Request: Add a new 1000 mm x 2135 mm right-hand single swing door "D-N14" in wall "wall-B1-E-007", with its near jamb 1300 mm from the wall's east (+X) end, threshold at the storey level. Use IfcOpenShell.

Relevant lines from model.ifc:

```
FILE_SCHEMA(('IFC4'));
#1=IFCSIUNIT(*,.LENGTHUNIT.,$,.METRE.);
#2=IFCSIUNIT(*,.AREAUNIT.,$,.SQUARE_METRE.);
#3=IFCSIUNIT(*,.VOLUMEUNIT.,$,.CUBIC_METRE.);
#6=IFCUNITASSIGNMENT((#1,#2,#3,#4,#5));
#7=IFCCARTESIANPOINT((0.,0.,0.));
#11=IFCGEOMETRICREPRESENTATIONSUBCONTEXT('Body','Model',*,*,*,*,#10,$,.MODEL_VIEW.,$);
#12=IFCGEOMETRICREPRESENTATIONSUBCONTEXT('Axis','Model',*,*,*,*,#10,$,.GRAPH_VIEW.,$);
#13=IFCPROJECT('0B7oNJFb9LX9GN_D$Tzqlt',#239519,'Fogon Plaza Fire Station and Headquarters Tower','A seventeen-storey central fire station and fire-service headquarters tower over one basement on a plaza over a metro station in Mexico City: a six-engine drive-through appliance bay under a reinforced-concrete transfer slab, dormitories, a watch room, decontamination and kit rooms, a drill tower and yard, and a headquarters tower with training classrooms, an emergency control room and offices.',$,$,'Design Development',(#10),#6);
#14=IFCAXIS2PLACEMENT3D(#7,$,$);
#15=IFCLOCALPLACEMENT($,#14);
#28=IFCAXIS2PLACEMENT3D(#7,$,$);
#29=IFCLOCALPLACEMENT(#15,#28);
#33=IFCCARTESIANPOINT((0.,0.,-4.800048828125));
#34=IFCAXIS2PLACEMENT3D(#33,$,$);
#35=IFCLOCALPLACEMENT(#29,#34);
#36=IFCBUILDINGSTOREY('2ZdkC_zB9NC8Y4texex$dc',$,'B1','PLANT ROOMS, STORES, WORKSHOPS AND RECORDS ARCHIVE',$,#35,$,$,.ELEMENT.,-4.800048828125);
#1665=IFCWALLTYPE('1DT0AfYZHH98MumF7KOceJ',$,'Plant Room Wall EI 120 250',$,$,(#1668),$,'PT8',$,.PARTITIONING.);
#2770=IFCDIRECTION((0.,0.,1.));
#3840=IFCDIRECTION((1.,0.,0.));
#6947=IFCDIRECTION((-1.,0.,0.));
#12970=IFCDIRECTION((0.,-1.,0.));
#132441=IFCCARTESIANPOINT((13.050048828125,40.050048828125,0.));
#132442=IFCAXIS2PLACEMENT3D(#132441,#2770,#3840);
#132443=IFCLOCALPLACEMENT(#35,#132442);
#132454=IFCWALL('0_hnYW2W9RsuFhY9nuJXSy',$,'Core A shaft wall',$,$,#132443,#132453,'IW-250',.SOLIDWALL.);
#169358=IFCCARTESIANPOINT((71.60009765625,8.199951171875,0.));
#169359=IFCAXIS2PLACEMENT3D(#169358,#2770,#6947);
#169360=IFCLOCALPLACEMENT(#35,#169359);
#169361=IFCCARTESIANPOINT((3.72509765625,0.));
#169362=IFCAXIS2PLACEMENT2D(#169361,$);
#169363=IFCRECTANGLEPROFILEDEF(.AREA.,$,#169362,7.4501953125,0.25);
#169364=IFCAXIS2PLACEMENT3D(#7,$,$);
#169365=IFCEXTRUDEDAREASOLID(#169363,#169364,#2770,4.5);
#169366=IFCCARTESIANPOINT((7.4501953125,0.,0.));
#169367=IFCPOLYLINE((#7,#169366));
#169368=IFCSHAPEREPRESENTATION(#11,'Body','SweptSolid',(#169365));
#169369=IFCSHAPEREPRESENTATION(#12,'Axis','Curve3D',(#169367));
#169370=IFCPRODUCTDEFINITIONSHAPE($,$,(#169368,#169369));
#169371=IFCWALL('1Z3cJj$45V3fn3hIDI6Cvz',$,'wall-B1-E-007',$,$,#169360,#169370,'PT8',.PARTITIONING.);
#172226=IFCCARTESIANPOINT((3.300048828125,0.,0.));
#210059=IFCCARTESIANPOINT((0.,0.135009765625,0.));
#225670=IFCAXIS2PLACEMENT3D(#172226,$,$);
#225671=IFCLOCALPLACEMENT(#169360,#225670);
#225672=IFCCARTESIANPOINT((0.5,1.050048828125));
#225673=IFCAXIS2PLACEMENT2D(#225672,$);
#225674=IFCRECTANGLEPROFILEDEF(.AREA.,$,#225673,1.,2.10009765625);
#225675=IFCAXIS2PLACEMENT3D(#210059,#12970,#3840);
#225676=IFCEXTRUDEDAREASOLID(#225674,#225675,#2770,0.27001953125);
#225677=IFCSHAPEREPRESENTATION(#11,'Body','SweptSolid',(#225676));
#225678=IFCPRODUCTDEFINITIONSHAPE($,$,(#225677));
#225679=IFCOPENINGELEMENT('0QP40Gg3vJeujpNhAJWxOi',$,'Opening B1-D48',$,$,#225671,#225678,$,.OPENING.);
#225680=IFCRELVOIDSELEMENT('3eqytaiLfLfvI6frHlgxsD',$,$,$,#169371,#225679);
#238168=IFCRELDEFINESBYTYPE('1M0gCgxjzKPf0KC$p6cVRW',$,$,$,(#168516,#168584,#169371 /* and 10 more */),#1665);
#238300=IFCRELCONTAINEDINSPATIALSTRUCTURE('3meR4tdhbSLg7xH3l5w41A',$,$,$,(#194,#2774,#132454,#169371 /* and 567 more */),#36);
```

```python
import numpy as np
import ifcopenshell
import ifcopenshell.api.feature
import ifcopenshell.api.geometry
import ifcopenshell.api.root
import ifcopenshell.api.spatial
import ifcopenshell.geom
import ifcopenshell.util.element
import ifcopenshell.util.placement
import ifcopenshell.util.representation
import ifcopenshell.util.shape
import ifcopenshell.util.unit

model = ifcopenshell.open("model.ifc")
unit_scale = ifcopenshell.util.unit.calculate_unit_scale(model)
settings = ifcopenshell.geom.settings()


def volume(element):
    """Net volume in cubic metres, openings subtracted."""
    shape = ifcopenshell.geom.create_shape(settings, element)
    return ifcopenshell.util.shape.get_volume(shape.geometry)


wall = model.by_guid("1Z3cJj$45V3fn3hIDI6Cvz")
storey = ifcopenshell.util.element.get_container(wall, ifc_class="IfcBuildingStorey")
context = ifcopenshell.util.representation.get_context(model, "Model", "Body", "MODEL_VIEW")
before = volume(wall)

width, height, from_end, sill = 1, 2.135, 1.3, 0.0  # metres

# The wall runs along its own X axis, and the end named is its -X end.
wall_shape = ifcopenshell.geom.create_shape(settings, wall)
x, y, z = ifcopenshell.util.shape.get_vertices(wall_shape.geometry).T
start = x.min() + from_end
face, thickness = float(y.min()), float(y.max() - y.min())
wall_matrix = ifcopenshell.util.placement.get_local_placement(wall.ObjectPlacement)
level = ifcopenshell.util.placement.get_local_placement(storey.ObjectPlacement)[2, 3]


def in_wall(x, y):
    """Placement at x, y metres in the wall's axes, at sill height."""
    matrix = wall_matrix.copy()
    matrix[:, 3] = wall_matrix @ np.array([x / unit_scale, y / unit_scale, 0.0, 1.0])
    matrix[2, 3] = level + sill / unit_scale
    return matrix


# Opening: a box that overshoots both wall faces by 50 mm.
opening = ifcopenshell.api.root.create_entity(model, ifc_class="IfcOpeningElement", predefined_type="OPENING")
box = ifcopenshell.api.geometry.add_wall_representation(
    model, context=context, length=width, height=height, thickness=thickness + 0.1
)
ifcopenshell.api.geometry.assign_representation(model, product=opening, representation=box)
ifcopenshell.api.geometry.edit_object_placement(model, product=opening, matrix=in_wall(start, face - 0.05), is_si=False)
ifcopenshell.api.feature.add_feature(model, feature=opening, element=wall)

door = ifcopenshell.api.root.create_entity(model, ifc_class="IfcDoor", name="D-N14", predefined_type="DOOR")
door.OverallWidth, door.OverallHeight = width / unit_scale, height / unit_scale
door.OperationType = "SINGLE_SWING_RIGHT"
body = ifcopenshell.api.geometry.add_door_representation(
    model,
    context=context,
    overall_width=door.OverallWidth,
    overall_height=door.OverallHeight,
    operation_type="SINGLE_SWING_RIGHT",
    lining_properties={"LiningDepth": thickness / unit_scale, "ThresholdDepth": thickness / unit_scale},
)
ifcopenshell.api.geometry.assign_representation(model, product=door, representation=body)
ifcopenshell.api.spatial.assign_container(model, products=[door], relating_structure=storey)
ifcopenshell.api.feature.add_filling(model, opening=opening, element=door)

# The lining spans the wall, so the door starts at the wall face.
ifcopenshell.api.geometry.edit_object_placement(model, product=door, matrix=in_wall(start, face), is_si=False)

after = volume(wall)

print(f"wall volume {before:.3f} -> {after:.3f} m3")

model.write("model_v2.ifc")
```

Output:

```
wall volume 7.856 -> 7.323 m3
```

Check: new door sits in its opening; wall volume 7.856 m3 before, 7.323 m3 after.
